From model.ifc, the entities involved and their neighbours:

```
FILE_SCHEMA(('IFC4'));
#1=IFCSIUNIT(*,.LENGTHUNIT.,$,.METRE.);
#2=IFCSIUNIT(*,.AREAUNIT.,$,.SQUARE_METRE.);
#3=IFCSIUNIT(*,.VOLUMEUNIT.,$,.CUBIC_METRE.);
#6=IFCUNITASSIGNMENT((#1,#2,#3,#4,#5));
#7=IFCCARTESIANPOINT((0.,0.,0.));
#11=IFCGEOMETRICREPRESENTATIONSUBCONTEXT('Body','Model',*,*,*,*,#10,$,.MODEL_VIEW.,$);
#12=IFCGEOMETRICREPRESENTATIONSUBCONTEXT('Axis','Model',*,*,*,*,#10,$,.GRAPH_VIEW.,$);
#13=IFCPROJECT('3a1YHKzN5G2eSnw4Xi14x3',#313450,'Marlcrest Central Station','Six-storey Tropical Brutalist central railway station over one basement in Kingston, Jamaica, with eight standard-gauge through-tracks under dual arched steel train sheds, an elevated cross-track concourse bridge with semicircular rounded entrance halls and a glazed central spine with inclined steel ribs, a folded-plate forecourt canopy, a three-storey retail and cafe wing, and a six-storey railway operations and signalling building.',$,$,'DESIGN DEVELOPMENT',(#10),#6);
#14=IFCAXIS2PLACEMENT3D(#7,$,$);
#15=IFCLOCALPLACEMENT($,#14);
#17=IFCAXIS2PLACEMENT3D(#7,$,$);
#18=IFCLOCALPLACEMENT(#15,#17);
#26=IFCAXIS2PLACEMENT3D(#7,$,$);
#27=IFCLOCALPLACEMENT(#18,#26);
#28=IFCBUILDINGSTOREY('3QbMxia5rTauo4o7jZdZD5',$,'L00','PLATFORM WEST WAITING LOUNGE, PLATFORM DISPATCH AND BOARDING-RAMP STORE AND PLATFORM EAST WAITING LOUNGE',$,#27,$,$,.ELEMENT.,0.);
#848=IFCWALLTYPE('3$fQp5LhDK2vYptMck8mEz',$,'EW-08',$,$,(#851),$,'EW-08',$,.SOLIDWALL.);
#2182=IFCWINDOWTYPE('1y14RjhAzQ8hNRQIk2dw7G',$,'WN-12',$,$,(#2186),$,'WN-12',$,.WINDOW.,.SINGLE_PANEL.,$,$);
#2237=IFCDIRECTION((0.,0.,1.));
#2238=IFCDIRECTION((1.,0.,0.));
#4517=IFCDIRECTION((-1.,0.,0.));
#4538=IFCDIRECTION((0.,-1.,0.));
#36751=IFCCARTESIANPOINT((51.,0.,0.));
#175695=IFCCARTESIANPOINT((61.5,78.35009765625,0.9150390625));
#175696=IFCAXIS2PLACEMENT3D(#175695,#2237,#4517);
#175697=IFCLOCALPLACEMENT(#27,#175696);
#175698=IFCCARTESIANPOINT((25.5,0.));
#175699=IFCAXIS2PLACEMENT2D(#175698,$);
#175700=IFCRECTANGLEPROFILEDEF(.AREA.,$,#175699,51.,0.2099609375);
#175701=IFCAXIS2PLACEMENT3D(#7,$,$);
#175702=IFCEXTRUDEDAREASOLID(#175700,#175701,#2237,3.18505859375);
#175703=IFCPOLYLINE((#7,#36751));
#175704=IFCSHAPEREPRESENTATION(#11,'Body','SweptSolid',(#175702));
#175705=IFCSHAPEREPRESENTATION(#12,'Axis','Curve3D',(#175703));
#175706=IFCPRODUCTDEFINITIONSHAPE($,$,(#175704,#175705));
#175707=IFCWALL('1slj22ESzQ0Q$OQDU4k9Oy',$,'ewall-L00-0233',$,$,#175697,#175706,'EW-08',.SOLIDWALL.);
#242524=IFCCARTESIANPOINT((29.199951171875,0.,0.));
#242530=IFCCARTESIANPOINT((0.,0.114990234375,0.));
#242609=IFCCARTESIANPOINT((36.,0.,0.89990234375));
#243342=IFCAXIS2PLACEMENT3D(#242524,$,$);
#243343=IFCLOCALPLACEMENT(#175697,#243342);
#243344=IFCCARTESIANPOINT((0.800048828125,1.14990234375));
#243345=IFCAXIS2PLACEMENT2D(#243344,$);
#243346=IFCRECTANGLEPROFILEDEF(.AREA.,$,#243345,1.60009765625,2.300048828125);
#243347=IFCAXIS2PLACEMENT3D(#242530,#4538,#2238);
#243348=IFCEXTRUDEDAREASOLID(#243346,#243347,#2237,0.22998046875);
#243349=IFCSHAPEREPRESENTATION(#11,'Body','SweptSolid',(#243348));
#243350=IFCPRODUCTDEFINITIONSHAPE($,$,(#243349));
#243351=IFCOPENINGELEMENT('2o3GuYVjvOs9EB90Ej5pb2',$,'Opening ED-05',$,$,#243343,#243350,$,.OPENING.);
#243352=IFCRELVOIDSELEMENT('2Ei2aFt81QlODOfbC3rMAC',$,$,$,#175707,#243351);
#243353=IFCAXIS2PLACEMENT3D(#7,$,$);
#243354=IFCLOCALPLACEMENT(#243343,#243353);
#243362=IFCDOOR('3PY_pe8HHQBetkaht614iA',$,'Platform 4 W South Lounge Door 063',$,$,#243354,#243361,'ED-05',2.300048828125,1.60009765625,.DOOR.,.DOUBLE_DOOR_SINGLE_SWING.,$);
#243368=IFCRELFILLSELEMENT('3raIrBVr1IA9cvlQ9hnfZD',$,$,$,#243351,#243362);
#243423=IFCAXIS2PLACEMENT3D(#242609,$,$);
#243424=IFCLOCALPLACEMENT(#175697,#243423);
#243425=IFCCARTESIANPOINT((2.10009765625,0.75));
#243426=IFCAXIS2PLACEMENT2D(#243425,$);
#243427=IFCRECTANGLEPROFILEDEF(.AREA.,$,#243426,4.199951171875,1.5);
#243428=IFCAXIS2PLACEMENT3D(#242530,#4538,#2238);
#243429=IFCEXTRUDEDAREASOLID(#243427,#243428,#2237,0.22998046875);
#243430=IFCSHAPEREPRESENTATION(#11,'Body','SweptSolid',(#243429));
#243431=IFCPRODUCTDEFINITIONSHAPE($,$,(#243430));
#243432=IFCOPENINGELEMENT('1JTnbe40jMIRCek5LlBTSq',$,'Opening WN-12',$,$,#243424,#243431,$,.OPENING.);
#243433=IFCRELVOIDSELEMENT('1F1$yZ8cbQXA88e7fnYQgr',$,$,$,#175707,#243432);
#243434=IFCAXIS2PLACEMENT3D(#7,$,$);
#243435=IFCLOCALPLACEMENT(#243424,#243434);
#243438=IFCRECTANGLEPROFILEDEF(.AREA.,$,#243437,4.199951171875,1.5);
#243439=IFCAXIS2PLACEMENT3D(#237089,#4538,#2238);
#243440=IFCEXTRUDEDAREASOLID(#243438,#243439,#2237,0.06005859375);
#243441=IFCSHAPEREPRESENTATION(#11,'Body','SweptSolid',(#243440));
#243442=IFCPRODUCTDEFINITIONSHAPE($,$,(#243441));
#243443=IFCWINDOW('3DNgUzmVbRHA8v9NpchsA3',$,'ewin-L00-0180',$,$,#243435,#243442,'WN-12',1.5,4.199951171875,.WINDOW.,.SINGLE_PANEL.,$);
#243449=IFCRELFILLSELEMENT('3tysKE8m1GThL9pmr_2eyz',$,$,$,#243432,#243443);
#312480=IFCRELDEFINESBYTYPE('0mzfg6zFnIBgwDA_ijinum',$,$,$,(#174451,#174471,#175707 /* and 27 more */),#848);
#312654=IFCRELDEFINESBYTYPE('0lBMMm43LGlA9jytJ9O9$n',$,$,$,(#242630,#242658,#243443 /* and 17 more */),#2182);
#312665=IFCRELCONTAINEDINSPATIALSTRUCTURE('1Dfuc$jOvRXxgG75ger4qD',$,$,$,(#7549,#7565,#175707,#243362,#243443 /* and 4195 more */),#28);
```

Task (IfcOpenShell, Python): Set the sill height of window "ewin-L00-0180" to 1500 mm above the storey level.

```python
import numpy as np
import ifcopenshell
import ifcopenshell.api.geometry
import ifcopenshell.geom
import ifcopenshell.util.element
import ifcopenshell.util.placement
import ifcopenshell.util.shape
import ifcopenshell.util.unit

model = ifcopenshell.open("model.ifc")
unit_scale = ifcopenshell.util.unit.calculate_unit_scale(model)

window = model.by_guid("3DNgUzmVbRHA8v9NpchsA3")
opening = window.FillsVoids[0].RelatingOpeningElement
storey = ifcopenshell.util.element.get_container(window, ifc_class="IfcBuildingStorey")
level = ifcopenshell.util.placement.get_local_placement(storey.ObjectPlacement)[2, 3]

# The opening's origin need not be at the sill, so measure its lowest point.
shape = ifcopenshell.geom.create_shape(ifcopenshell.geom.settings(), opening)
bottom = ifcopenshell.util.shape.get_shape_bottom_elevation(shape, shape.geometry) / unit_scale
dz = level + 1.5 - bottom

shift = np.array([0.0, 0.0, dz])
# The window is placed relative to its opening, so it follows when the opening moves.
matrix = ifcopenshell.util.placement.get_local_placement(opening.ObjectPlacement)
matrix[:3, 3] += shift
ifcopenshell.api.geometry.edit_object_placement(
    model, product=opening, matrix=matrix, is_si=False, should_transform_children=True
)

print(f"moved by {dz * unit_scale:+.3f} m")

model.write("model_updated.ifc")
```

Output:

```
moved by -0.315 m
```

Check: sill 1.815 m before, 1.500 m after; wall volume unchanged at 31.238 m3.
